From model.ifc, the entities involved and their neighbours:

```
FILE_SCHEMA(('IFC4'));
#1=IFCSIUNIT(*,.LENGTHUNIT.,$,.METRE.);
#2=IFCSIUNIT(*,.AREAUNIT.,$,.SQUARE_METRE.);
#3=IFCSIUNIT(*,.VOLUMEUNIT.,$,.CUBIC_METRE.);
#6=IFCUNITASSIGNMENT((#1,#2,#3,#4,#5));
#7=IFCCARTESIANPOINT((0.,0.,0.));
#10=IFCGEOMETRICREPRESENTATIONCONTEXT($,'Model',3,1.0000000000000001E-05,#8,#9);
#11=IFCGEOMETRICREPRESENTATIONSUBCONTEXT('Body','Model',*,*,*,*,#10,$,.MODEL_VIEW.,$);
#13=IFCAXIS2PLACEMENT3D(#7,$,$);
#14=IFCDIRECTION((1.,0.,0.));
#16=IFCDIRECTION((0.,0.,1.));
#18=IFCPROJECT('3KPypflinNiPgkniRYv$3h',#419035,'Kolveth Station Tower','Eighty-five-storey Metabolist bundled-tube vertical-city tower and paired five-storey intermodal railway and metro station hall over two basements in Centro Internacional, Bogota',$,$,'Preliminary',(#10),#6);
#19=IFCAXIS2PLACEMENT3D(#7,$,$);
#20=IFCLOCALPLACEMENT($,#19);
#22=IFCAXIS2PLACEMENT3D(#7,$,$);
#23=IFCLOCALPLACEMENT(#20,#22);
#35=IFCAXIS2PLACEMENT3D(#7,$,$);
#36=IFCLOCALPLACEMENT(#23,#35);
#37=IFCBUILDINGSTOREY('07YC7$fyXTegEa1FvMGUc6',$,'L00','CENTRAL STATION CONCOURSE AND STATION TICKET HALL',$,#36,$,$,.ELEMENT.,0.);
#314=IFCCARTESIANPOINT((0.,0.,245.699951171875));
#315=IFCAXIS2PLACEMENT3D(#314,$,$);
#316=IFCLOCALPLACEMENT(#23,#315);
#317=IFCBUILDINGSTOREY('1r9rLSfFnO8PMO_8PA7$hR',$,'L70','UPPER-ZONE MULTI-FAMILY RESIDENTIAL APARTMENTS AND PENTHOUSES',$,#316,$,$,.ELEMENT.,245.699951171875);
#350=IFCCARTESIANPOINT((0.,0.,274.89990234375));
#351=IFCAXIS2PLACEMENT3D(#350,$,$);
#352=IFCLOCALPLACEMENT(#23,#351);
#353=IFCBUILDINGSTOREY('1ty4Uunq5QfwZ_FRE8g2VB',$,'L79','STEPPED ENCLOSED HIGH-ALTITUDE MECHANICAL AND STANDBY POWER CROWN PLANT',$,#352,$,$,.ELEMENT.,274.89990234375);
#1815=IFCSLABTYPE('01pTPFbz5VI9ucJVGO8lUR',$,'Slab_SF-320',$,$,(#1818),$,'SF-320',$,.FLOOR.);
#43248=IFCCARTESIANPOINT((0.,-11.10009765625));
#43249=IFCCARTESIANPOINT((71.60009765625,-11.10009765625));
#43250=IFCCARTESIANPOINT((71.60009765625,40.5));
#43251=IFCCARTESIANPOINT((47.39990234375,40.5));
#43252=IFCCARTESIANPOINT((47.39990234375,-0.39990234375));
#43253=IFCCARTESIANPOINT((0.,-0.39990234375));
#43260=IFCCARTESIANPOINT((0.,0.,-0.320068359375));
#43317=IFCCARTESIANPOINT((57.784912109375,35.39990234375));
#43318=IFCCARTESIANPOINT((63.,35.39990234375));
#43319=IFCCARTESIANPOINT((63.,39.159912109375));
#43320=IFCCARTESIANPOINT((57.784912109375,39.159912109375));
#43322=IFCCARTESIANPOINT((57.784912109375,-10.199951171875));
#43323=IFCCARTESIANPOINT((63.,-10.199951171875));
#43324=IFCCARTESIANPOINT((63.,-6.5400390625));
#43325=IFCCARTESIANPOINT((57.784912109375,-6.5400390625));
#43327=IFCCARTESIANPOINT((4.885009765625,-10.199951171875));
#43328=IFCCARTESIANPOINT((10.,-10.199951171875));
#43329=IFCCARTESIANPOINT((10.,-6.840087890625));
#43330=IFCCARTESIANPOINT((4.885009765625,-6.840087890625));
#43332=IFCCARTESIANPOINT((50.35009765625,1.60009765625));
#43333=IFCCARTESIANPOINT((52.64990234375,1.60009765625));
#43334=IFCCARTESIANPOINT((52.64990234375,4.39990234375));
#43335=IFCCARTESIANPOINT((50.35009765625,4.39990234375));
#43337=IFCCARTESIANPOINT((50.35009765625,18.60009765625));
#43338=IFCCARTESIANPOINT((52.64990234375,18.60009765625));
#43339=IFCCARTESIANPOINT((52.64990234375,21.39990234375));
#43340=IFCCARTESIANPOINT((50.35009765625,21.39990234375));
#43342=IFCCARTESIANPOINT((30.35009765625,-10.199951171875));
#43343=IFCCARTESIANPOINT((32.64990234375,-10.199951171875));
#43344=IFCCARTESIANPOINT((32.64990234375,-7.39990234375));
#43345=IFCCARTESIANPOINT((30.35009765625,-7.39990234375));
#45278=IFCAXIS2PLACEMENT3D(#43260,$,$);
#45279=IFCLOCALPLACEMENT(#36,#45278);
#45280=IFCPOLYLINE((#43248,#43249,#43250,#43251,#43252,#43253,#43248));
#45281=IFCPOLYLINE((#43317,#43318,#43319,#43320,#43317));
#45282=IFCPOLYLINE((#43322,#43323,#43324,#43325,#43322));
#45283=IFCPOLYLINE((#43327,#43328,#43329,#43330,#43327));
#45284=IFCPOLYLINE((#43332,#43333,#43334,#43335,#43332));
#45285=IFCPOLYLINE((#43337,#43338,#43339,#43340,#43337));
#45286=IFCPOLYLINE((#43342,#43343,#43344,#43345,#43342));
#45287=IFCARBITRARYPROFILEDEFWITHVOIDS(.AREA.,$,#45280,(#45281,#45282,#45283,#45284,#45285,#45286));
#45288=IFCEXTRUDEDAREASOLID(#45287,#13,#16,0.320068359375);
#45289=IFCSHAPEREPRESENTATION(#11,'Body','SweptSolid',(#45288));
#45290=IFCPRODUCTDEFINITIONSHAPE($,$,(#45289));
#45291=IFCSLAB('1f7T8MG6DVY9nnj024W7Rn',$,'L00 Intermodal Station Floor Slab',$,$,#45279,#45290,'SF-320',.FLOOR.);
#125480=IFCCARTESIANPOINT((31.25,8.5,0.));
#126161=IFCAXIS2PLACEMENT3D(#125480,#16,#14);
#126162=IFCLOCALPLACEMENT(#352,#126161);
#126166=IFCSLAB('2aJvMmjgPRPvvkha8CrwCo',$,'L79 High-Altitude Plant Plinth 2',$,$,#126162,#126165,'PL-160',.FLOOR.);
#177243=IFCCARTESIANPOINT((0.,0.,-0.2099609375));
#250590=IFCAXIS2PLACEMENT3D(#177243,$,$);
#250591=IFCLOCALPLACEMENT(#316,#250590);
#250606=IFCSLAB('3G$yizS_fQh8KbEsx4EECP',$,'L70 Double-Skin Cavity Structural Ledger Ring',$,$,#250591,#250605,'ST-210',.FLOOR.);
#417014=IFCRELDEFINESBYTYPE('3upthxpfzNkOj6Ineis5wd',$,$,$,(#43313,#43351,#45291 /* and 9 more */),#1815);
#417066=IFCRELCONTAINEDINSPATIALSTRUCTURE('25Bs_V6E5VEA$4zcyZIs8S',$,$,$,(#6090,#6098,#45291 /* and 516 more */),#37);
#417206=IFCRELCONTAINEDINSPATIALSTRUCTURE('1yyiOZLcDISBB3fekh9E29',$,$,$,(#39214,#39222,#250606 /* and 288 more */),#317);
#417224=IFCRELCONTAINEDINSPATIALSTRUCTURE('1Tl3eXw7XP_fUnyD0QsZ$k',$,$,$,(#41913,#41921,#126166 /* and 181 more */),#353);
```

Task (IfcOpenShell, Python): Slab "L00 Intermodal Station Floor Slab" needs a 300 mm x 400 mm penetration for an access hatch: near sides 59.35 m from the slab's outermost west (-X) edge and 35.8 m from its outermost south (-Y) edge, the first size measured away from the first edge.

```python
import numpy as np
import ifcopenshell
import ifcopenshell.api.feature
import ifcopenshell.api.geometry
import ifcopenshell.api.root
import ifcopenshell.geom
import ifcopenshell.util.placement
import ifcopenshell.util.representation
import ifcopenshell.util.shape
import ifcopenshell.util.unit

model = ifcopenshell.open("model.ifc")
unit_scale = ifcopenshell.util.unit.calculate_unit_scale(model)
settings = ifcopenshell.geom.settings()


def volume(element):
    """Net volume in cubic metres, openings subtracted."""
    shape = ifcopenshell.geom.create_shape(settings, element)
    return ifcopenshell.util.shape.get_volume(shape.geometry)


slab = model.by_guid("1f7T8MG6DVY9nnj024W7Rn")
before = volume(slab)

# Extent in the slab's own axes, in metres. The edges named are its -X and -Y sides.
slab_shape = ifcopenshell.geom.create_shape(settings, slab)
vertices = ifcopenshell.util.shape.get_vertices(slab_shape.geometry)
x_min, y_min, bottom = vertices.min(axis=0)
top = vertices[:, 2].max()

opening = ifcopenshell.api.root.create_entity(model, ifc_class="IfcOpeningElement", name="Access hatch opening", predefined_type="OPENING")
context = ifcopenshell.util.representation.get_context(model, "Model", "Body", "MODEL_VIEW")
width, depth = 0.3, 0.4
outline = [(0.0, 0.0), (width, 0.0), (width, depth), (0.0, depth), (0.0, 0.0)]
# Overshoot both faces by 50 mm so the cut is clean.
shape = ifcopenshell.api.geometry.add_slab_representation(
    model, context=context, depth=top - bottom + 0.1, polyline=outline
)
ifcopenshell.api.geometry.assign_representation(model, product=opening, representation=shape)

matrix = ifcopenshell.util.placement.get_local_placement(slab.ObjectPlacement)
matrix[:, 3] = matrix @ np.append(np.array([x_min + 59.35, y_min + 35.8, bottom - 0.05]) / unit_scale, 1.0)
ifcopenshell.api.geometry.edit_object_placement(model, product=opening, matrix=matrix, is_si=False)
ifcopenshell.api.feature.add_feature(model, feature=opening, element=slab)

after = volume(slab)

print(f"slab volume {before:.3f} -> {after:.3f} m3")

model.write("model-out.ifc")
```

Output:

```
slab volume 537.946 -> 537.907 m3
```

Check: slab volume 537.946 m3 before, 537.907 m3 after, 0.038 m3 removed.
